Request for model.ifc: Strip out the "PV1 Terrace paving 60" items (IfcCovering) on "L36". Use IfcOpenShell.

First a look at what the model holds.

```python
import ifcopenshell
import ifcopenshell.util.element

model = ifcopenshell.open("model.ifc")
print(model.schema)
storey = next(s for s in model.by_type("IfcBuildingStorey") if s.Name == "L36")
coverings = [e for e in ifcopenshell.util.element.get_decomposition(storey) if e.is_a("IfcCovering")]
seen = {}
for e in coverings:
    element_type = ifcopenshell.util.element.get_type(e)
    name = element_type.Name if element_type not in (None, e) else None
    seen[name] = seen.get(name, 0) + 1
for name, count in sorted(seen.items(), key=str):
    print(count, "x", name)
```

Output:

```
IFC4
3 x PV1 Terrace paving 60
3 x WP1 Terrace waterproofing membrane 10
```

```python
import ifcopenshell
import ifcopenshell.api.root
import ifcopenshell.util.element

model = ifcopenshell.open("model.ifc")

storey = next(s for s in model.by_type("IfcBuildingStorey") if s.Name == "L36")
coverings = [e for e in ifcopenshell.util.element.get_decomposition(storey) if e.is_a("IfcCovering")]
targets = [e for e in coverings if (t := ifcopenshell.util.element.get_type(e)) not in (None, e) and t.Name == "PV1 Terrace paving 60"]

for e in targets:
    ifcopenshell.api.root.remove_product(model, product=e)
print(len(targets), "removed")

model.write("model-out.ifc")
```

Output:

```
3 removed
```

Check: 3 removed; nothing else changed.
